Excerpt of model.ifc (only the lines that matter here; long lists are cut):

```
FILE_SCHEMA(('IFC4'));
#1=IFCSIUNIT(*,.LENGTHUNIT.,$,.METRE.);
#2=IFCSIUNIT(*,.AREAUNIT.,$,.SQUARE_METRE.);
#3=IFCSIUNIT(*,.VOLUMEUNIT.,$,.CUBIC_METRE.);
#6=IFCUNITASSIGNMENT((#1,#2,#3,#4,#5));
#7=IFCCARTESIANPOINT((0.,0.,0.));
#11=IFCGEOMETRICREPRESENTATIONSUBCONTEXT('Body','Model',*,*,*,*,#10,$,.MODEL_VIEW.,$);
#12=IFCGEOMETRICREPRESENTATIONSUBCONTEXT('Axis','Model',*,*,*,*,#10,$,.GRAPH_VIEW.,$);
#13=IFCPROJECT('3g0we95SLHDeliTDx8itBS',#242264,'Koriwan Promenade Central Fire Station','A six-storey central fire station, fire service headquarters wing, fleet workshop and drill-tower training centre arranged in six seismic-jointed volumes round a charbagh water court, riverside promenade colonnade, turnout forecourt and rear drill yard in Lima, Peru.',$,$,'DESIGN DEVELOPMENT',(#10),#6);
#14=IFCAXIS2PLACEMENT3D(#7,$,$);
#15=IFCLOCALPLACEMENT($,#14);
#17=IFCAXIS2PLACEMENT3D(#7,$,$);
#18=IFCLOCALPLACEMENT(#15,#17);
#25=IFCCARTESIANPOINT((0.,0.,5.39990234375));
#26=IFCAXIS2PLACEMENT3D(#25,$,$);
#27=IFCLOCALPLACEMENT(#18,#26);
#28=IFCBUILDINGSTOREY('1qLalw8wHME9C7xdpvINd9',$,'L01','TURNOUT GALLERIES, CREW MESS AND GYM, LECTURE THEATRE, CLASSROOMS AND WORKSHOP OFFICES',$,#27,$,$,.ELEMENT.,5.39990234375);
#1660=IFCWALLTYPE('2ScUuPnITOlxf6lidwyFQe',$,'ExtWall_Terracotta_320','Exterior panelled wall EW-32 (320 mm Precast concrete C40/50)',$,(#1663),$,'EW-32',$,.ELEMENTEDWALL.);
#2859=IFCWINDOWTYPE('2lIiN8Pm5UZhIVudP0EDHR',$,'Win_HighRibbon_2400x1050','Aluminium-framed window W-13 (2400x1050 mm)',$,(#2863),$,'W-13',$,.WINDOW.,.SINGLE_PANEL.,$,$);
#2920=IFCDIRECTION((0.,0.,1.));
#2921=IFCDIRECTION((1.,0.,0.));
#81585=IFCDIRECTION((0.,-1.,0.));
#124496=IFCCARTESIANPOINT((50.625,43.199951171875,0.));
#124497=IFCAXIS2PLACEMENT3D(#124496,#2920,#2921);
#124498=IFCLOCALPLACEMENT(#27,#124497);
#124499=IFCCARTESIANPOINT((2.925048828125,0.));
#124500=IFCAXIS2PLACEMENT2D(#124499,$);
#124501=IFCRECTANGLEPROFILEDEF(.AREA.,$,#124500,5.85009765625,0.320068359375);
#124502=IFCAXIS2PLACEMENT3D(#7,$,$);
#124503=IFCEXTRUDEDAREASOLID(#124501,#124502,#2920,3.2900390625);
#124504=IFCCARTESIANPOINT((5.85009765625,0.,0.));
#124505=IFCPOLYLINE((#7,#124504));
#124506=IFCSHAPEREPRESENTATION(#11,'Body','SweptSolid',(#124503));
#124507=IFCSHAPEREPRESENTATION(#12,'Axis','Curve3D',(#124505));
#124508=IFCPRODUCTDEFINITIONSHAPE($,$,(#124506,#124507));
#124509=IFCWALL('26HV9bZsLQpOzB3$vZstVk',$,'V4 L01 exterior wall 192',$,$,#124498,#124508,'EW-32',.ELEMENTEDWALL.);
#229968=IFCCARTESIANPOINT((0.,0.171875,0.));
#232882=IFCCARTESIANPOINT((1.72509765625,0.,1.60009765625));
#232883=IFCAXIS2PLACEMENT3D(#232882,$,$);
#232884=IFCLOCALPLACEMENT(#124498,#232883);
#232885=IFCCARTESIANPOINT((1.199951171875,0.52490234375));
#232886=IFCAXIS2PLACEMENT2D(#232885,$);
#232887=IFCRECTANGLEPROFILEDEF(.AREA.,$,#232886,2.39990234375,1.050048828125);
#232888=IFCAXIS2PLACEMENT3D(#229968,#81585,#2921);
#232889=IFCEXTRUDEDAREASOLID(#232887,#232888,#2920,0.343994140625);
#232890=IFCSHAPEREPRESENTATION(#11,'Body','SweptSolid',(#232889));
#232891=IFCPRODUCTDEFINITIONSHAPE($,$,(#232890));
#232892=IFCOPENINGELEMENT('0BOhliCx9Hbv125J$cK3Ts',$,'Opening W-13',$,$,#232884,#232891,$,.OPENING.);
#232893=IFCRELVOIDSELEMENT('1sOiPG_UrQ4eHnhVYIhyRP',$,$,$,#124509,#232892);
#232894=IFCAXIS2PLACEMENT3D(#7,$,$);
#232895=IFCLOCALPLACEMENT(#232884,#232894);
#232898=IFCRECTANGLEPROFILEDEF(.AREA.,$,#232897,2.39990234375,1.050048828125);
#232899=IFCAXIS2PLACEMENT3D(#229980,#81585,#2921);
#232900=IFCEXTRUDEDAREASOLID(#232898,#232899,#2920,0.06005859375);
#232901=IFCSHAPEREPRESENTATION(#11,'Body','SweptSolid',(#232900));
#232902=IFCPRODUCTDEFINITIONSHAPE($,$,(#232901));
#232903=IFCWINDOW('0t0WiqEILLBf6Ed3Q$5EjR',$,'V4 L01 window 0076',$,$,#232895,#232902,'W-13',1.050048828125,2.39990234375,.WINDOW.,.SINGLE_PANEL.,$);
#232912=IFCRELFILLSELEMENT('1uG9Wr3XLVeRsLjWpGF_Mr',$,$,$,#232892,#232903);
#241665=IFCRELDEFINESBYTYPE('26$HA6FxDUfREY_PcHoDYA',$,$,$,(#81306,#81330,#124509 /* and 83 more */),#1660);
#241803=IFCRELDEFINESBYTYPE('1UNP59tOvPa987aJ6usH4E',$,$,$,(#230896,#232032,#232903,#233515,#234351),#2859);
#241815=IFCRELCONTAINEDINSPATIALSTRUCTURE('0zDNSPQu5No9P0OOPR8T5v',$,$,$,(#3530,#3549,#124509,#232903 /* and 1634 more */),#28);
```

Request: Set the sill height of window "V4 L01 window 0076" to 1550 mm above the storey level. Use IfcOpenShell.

```python
import numpy as np
import ifcopenshell
import ifcopenshell.api.geometry
import ifcopenshell.geom
import ifcopenshell.util.element
import ifcopenshell.util.placement
import ifcopenshell.util.shape
import ifcopenshell.util.unit

model = ifcopenshell.open("model.ifc")
unit_scale = ifcopenshell.util.unit.calculate_unit_scale(model)

window = model.by_id(232903)
opening = window.FillsVoids[0].RelatingOpeningElement
storey = ifcopenshell.util.element.get_container(window, ifc_class="IfcBuildingStorey")
level = ifcopenshell.util.placement.get_local_placement(storey.ObjectPlacement)[2, 3]

# The opening's origin need not be at the sill, so measure its lowest point.
shape = ifcopenshell.geom.create_shape(ifcopenshell.geom.settings(), opening)
bottom = ifcopenshell.util.shape.get_shape_bottom_elevation(shape, shape.geometry) / unit_scale
dz = level + 1.55 - bottom

shift = np.array([0.0, 0.0, dz])
# The window is placed relative to its opening, so it follows when the opening moves.
matrix = ifcopenshell.util.placement.get_local_placement(opening.ObjectPlacement)
matrix[:3, 3] += shift
ifcopenshell.api.geometry.edit_object_placement(
    model, product=opening, matrix=matrix, is_si=False, should_transform_children=True
)

print(f"moved by {dz * unit_scale:+.3f} m")

model.write("model_rev.ifc")
```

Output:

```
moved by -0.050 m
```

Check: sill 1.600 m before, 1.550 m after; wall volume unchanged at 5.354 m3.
